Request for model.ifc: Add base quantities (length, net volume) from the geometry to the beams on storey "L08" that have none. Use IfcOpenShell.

First a look at what the model holds.

```python
import ifcopenshell
import ifcopenshell.util.element
import ifcopenshell.util.unit

model = ifcopenshell.open("model.ifc")
print(model.schema)
for unit_type in ("LENGTHUNIT", "AREAUNIT", "VOLUMEUNIT"):
    print(unit_type, ifcopenshell.util.unit.calculate_unit_scale(model, unit_type))
storey = next(s for s in model.by_type("IfcBuildingStorey") if s.Name == "L08")
beams = [e for e in ifcopenshell.util.element.get_decomposition(storey) if e.is_a("IfcBeam")]
for e in sorted(beams, key=lambda e: e.id()):
    print(e.id(), e.is_a(), e.Name, list(ifcopenshell.util.element.get_psets(e, qtos_only=True)), sep=" | ")
```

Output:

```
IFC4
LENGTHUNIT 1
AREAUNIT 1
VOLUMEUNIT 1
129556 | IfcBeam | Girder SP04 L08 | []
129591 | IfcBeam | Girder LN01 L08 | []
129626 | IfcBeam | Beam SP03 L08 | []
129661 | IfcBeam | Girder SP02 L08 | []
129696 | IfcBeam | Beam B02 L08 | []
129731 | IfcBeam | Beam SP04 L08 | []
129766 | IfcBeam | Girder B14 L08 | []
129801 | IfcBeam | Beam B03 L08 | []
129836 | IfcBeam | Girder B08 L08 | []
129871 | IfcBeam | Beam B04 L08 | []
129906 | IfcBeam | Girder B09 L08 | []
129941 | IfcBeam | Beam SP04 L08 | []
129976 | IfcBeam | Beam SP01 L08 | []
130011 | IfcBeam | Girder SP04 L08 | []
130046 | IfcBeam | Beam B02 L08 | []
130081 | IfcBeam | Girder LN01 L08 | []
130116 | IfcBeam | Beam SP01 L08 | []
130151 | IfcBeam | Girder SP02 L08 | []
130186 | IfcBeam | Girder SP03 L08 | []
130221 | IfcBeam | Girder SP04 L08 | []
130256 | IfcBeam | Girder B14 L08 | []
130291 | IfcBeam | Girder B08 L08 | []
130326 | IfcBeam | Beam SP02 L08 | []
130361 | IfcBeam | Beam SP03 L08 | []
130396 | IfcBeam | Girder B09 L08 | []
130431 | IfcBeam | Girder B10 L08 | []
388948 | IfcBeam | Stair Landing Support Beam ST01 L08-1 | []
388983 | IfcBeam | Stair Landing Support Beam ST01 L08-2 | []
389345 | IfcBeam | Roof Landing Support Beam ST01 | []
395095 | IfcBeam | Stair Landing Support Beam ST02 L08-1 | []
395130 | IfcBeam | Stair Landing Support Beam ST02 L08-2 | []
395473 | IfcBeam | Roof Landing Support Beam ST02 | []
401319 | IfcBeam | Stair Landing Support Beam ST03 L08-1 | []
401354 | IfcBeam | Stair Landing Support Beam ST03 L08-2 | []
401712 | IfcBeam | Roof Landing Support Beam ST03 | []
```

```python
import ifcopenshell
import ifcopenshell.api.pset
import ifcopenshell.geom
import ifcopenshell.util.element
import ifcopenshell.util.shape
import ifcopenshell.util.unit

model = ifcopenshell.open("model.ifc")
unit_scale = ifcopenshell.util.unit.calculate_unit_scale(model)
volume_scale = ifcopenshell.util.unit.calculate_unit_scale(model, "VOLUMEUNIT")
settings = ifcopenshell.geom.settings()

storey = next(s for s in model.by_type("IfcBuildingStorey") if s.Name == "L08")
beams = [e for e in ifcopenshell.util.element.get_decomposition(storey) if e.is_a("IfcBeam")]

for e in sorted(beams, key=lambda e: e.id()):
    if ifcopenshell.util.element.get_psets(e, qtos_only=True, should_inherit=False):
        continue
    # Geometry comes back in metres, in the element's own axes.
    shape = ifcopenshell.geom.create_shape(settings, e)
    values = {
        "Length": ifcopenshell.util.shape.get_max_xyz(shape.geometry) / unit_scale,
        "NetVolume": ifcopenshell.util.shape.get_volume(shape.geometry) / volume_scale,
    }
    qto = ifcopenshell.api.pset.add_qto(model, product=e, name="Qto_BeamBaseQuantities")
    ifcopenshell.api.pset.edit_qto(model, qto=qto, properties=values)
    print(e.id(), {k: round(v, 3) for k, v in values.items()})

model.write("model_v2.ifc")
```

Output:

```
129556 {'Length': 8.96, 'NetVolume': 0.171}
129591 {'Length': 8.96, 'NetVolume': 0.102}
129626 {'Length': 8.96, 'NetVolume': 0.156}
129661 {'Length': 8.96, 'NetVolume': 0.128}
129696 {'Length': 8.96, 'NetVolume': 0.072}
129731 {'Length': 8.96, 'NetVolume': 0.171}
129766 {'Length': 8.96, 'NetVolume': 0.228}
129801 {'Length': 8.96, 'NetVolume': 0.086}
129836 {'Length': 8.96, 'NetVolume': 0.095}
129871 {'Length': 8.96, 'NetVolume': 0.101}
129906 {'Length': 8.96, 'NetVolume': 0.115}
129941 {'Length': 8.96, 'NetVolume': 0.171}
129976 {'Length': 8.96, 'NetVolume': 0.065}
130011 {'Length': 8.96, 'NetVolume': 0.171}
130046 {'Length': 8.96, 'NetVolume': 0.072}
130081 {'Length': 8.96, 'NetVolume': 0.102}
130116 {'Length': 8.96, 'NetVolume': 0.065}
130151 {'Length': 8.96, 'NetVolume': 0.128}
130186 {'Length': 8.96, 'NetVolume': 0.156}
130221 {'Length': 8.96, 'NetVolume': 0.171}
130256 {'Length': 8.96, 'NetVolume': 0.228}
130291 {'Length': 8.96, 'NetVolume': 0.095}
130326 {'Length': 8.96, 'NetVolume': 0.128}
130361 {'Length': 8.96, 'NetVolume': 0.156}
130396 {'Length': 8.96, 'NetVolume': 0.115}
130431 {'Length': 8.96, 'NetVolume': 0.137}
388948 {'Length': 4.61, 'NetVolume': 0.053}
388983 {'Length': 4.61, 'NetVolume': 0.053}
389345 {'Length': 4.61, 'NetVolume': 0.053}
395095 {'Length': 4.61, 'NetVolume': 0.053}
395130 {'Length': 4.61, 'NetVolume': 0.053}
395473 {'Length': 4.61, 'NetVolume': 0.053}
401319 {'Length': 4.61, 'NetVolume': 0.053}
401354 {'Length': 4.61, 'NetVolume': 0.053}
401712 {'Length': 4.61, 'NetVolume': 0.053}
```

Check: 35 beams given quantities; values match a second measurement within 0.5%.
